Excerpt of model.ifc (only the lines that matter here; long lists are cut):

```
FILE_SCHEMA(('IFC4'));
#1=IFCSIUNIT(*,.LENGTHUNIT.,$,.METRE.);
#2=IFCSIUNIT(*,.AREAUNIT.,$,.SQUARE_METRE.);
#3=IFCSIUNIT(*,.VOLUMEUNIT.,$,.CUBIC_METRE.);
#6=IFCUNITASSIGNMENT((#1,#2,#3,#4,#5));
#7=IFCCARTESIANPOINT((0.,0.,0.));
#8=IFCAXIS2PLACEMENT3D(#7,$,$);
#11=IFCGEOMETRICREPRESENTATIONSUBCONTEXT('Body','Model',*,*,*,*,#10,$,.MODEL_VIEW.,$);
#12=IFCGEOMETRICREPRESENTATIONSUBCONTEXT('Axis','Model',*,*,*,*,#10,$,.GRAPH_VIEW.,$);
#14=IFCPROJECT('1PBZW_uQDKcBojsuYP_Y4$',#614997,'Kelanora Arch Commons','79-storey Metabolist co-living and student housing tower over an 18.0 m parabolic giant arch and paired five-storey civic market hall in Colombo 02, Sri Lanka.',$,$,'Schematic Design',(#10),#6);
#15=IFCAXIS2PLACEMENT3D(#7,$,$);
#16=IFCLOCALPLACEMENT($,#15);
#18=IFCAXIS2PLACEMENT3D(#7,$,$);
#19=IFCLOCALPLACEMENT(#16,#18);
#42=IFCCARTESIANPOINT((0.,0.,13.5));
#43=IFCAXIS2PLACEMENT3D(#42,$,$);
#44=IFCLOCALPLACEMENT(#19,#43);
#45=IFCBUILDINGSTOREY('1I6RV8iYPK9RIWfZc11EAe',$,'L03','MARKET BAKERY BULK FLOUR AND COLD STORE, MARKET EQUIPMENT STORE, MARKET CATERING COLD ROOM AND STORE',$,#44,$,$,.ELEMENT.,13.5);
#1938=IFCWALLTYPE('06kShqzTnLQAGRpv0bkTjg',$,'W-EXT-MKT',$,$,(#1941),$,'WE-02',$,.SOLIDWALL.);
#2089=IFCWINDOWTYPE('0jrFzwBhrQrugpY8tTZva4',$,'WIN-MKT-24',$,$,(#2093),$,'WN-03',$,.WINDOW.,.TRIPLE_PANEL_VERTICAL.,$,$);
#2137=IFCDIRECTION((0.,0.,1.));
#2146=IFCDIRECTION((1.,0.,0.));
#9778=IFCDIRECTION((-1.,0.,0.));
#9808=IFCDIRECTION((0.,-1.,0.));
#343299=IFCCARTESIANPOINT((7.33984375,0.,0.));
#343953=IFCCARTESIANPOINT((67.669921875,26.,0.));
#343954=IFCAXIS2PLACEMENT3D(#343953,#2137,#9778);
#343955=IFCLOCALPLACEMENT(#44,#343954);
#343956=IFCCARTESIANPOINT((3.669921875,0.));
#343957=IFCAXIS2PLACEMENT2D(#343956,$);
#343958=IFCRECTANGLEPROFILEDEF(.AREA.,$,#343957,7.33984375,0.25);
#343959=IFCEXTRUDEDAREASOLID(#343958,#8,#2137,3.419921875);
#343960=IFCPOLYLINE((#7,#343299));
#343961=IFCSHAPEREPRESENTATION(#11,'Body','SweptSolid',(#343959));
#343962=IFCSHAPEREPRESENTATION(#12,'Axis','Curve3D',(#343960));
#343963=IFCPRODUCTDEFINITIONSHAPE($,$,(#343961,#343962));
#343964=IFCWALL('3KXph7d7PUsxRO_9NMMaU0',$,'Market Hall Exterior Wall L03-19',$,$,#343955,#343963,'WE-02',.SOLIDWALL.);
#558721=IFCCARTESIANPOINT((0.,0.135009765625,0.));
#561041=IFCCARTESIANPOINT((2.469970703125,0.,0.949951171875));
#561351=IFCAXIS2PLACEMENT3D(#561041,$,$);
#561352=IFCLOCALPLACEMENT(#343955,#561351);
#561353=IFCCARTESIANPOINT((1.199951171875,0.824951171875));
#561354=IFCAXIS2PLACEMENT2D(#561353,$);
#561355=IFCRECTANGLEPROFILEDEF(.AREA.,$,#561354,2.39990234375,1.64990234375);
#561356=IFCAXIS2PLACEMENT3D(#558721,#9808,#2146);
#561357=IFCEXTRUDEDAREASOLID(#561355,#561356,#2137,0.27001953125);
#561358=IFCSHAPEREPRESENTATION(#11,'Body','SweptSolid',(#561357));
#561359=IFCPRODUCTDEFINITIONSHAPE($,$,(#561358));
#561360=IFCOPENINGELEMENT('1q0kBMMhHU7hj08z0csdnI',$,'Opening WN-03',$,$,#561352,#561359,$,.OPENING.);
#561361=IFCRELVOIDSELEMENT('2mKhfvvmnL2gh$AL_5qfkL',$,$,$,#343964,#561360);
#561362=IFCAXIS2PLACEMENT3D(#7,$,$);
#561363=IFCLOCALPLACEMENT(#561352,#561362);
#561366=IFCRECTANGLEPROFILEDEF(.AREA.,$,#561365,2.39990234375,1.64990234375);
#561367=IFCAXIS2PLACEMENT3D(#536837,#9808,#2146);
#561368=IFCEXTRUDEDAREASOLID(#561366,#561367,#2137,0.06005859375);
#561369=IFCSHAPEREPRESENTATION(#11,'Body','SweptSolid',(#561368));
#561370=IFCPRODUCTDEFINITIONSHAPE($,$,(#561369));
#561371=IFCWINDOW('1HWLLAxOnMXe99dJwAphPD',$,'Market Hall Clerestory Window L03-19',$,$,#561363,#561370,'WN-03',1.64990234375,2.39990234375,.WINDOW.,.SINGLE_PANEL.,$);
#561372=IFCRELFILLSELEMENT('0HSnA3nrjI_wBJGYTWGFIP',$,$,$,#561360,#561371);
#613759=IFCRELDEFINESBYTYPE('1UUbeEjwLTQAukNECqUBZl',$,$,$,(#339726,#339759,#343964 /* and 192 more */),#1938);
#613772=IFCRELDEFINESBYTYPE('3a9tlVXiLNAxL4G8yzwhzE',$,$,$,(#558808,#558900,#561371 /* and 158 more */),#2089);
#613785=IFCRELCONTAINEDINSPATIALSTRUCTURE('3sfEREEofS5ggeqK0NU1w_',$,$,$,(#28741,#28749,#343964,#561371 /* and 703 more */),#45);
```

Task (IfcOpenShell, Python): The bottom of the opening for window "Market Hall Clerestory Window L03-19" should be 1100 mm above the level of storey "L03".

```python
import numpy as np
import ifcopenshell
import ifcopenshell.api.geometry
import ifcopenshell.geom
import ifcopenshell.util.element
import ifcopenshell.util.placement
import ifcopenshell.util.shape
import ifcopenshell.util.unit

model = ifcopenshell.open("model.ifc")
unit_scale = ifcopenshell.util.unit.calculate_unit_scale(model)

window = model.by_guid("1HWLLAxOnMXe99dJwAphPD")
opening = window.FillsVoids[0].RelatingOpeningElement
storey = ifcopenshell.util.element.get_container(window, ifc_class="IfcBuildingStorey")
level = ifcopenshell.util.placement.get_local_placement(storey.ObjectPlacement)[2, 3]

# The opening's origin need not be at the sill, so measure its lowest point.
shape = ifcopenshell.geom.create_shape(ifcopenshell.geom.settings(), opening)
bottom = ifcopenshell.util.shape.get_shape_bottom_elevation(shape, shape.geometry) / unit_scale
dz = level + 1.1 / unit_scale - bottom

shift = np.array([0.0, 0.0, dz])
# The window is placed relative to its opening, so it follows when the opening moves.
matrix = ifcopenshell.util.placement.get_local_placement(opening.ObjectPlacement)
matrix[:3, 3] += shift
ifcopenshell.api.geometry.edit_object_placement(
    model, product=opening, matrix=matrix, is_si=False, should_transform_children=True
)

print(f"moved by {dz * unit_scale:+.3f} m")

model.write("model-out.ifc")
```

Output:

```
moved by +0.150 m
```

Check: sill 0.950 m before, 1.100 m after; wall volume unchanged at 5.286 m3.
